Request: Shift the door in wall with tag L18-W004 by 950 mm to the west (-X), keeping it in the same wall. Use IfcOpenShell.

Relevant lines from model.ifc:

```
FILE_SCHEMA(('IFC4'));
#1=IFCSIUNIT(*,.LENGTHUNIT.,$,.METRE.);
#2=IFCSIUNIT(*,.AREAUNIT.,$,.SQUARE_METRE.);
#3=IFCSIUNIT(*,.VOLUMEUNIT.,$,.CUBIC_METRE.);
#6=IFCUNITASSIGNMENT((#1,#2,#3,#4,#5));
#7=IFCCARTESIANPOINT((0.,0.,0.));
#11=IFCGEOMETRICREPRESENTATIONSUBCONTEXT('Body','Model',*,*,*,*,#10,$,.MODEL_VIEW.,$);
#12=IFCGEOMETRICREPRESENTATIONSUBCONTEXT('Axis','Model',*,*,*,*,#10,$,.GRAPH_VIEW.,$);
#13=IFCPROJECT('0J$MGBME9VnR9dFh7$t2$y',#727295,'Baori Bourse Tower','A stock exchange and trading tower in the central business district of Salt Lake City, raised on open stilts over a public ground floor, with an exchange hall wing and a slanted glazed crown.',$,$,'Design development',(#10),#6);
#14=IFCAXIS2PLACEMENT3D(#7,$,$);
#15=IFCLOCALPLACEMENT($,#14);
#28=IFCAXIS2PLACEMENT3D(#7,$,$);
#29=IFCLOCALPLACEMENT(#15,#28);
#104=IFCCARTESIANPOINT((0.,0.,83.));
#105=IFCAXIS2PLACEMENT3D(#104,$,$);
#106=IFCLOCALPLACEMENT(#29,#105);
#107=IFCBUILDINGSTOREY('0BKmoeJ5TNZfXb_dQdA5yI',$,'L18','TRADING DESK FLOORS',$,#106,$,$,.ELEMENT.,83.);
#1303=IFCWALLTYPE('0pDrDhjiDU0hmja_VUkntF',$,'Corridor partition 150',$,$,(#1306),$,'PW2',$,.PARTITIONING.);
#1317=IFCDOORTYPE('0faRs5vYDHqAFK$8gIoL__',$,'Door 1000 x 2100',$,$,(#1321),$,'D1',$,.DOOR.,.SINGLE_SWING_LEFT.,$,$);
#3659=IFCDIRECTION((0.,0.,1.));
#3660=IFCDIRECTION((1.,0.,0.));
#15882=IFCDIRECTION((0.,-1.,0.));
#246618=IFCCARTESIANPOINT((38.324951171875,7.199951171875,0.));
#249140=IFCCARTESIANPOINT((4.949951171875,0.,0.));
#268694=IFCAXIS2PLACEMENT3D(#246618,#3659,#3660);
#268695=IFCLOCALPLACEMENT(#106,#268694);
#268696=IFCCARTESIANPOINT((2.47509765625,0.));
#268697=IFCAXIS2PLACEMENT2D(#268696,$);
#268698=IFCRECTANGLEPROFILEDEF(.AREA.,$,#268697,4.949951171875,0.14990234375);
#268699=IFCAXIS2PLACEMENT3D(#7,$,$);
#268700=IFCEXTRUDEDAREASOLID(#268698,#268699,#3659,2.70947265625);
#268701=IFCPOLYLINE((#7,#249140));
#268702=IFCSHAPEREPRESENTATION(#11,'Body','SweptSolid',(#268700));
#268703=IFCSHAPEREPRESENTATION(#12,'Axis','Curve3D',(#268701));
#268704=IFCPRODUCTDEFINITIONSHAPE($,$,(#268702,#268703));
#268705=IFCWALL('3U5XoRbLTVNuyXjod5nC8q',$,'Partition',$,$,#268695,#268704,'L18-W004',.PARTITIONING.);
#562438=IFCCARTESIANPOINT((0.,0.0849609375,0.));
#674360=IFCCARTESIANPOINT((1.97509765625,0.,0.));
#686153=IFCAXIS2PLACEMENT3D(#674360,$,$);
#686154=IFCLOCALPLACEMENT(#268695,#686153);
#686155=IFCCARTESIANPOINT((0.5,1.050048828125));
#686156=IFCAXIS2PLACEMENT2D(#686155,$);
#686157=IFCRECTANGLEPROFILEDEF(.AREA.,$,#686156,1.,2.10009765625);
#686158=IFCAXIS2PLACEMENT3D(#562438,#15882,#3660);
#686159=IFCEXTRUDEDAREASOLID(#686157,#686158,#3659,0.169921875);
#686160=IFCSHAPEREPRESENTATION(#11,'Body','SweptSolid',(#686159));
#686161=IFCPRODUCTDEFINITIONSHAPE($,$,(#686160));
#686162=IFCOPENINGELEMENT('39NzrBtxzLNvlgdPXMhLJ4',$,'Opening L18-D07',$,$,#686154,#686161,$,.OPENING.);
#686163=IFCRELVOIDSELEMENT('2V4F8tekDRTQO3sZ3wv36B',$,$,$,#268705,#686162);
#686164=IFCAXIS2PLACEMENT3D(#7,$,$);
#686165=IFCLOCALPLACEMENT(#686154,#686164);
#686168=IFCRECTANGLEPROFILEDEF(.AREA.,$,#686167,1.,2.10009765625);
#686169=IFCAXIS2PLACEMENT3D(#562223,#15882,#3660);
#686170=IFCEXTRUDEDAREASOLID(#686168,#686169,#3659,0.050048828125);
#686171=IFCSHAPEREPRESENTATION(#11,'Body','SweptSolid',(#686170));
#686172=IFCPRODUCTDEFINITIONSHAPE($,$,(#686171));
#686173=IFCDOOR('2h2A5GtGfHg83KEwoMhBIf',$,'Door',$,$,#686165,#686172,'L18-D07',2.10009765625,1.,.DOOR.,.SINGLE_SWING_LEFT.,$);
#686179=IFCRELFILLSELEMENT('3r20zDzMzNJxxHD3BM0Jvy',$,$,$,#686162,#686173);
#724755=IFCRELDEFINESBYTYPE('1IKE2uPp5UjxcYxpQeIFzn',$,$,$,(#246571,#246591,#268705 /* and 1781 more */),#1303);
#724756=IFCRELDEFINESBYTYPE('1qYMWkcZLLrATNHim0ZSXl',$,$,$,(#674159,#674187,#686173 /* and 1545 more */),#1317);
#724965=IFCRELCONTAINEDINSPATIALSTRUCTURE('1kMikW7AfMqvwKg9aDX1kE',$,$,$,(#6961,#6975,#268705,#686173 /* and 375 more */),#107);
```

```python
import ifcopenshell
import ifcopenshell.api.geometry
import ifcopenshell.util.placement

model = ifcopenshell.open("model.ifc")

door = model.by_guid("2h2A5GtGfHg83KEwoMhBIf")
opening = door.FillsVoids[0].RelatingOpeningElement
wall = opening.VoidsElements[0].RelatingBuildingElement

wall_matrix = ifcopenshell.util.placement.get_local_placement(wall.ObjectPlacement)
shift = wall_matrix[:3, 0] * -0.95
before = ifcopenshell.util.placement.get_local_placement(door.ObjectPlacement)[:3, 3].copy()

# The door is placed relative to its opening, so it follows when the opening moves.
matrix = ifcopenshell.util.placement.get_local_placement(opening.ObjectPlacement)
matrix[:3, 3] += shift
ifcopenshell.api.geometry.edit_object_placement(
    model, product=opening, matrix=matrix, is_si=False, should_transform_children=True
)

after = ifcopenshell.util.placement.get_local_placement(door.ObjectPlacement)[:3, 3]
print("door moved by", (after - before).round(3) + 0.0)

model.write("model_v2.ifc")
```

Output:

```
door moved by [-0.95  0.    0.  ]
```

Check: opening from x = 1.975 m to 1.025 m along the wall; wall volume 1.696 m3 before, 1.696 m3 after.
